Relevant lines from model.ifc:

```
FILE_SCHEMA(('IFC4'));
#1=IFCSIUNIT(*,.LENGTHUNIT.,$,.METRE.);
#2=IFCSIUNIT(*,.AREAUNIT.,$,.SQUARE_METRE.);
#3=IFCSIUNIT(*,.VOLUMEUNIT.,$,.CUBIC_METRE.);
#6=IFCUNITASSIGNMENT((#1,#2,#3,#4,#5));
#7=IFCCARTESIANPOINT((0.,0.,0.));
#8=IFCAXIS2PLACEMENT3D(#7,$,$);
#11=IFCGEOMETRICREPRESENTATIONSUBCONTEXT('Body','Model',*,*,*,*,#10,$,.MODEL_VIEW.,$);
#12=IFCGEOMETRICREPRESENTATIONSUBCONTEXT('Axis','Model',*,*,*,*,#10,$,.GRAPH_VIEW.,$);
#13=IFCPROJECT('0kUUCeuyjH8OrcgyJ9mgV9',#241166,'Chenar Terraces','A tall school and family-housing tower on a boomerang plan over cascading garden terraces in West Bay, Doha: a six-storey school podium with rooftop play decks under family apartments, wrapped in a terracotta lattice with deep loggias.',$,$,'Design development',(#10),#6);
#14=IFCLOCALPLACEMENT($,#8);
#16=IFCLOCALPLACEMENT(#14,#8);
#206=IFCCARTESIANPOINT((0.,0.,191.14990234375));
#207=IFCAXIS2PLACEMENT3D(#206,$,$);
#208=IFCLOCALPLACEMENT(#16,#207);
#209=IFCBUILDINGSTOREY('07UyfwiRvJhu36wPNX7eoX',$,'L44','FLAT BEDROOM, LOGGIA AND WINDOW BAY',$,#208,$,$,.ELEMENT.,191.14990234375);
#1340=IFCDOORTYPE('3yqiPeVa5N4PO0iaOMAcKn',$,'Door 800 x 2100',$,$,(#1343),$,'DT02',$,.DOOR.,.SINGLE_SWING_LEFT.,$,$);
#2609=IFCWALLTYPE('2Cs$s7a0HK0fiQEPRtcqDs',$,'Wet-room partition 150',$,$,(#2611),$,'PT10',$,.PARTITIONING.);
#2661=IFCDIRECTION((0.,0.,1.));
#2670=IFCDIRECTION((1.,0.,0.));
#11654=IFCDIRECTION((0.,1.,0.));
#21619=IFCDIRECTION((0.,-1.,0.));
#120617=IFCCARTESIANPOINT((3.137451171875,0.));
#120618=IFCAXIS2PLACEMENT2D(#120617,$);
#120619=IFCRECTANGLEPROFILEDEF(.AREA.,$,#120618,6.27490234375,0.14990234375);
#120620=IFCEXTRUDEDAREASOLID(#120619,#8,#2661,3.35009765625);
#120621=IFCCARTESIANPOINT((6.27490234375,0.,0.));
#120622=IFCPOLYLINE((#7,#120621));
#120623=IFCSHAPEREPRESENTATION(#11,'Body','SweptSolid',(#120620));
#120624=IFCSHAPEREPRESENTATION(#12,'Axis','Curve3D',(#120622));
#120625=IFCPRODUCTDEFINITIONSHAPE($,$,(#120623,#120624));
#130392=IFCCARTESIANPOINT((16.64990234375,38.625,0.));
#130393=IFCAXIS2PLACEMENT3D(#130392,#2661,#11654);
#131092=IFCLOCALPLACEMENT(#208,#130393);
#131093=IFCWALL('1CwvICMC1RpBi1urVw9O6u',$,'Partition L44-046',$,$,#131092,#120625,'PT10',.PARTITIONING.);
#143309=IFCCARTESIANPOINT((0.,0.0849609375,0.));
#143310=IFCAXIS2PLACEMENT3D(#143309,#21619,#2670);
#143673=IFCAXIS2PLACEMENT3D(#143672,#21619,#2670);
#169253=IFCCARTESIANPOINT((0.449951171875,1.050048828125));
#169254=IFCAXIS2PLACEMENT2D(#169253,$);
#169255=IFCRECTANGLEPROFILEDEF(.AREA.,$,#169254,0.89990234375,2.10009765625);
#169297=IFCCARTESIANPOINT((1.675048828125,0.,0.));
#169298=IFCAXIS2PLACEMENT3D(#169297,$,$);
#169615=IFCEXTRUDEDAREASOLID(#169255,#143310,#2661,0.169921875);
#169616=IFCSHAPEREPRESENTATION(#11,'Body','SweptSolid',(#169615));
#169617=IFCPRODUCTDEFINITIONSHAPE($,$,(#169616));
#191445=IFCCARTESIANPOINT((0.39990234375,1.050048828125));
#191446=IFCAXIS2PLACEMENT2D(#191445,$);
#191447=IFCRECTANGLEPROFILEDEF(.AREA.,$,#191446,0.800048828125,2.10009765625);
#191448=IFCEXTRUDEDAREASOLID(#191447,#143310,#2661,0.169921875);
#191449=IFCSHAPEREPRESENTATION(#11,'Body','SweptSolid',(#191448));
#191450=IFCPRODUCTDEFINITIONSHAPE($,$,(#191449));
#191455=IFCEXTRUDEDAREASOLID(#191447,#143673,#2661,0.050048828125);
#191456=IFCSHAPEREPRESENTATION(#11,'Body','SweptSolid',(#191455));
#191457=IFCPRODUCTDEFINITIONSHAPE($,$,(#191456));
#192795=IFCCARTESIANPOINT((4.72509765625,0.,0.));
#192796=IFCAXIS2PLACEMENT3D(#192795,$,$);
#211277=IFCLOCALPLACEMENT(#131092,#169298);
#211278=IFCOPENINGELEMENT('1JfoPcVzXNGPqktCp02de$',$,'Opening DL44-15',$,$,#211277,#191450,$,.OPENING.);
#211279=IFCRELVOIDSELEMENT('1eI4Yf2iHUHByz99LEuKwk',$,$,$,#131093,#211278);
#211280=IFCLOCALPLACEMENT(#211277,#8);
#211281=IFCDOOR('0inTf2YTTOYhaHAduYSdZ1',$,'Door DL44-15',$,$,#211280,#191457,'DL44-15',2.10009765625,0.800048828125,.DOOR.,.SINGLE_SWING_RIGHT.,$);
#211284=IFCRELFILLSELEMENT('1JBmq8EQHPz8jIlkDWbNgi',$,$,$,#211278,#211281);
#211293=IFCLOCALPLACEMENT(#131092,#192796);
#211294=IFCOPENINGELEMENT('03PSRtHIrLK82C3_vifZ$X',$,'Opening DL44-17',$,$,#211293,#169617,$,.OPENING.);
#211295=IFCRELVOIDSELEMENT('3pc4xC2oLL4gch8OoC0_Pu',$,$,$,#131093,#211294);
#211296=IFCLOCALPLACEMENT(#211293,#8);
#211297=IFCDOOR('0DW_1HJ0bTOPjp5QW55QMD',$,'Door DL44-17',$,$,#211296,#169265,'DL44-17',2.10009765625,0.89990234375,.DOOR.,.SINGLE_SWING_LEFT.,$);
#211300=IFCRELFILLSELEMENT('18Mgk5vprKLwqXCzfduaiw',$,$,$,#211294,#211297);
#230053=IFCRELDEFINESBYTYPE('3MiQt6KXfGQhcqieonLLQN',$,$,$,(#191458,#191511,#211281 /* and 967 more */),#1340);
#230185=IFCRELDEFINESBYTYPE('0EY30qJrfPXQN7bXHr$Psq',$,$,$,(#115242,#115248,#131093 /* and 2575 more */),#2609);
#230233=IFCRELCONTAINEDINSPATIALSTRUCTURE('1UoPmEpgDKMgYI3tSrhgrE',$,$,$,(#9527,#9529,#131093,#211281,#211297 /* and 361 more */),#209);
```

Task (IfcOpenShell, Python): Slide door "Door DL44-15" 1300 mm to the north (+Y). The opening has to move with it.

```python
import ifcopenshell
import ifcopenshell.api.geometry
import ifcopenshell.util.placement

model = ifcopenshell.open("model.ifc")

door = model.by_guid("0inTf2YTTOYhaHAduYSdZ1")
opening = door.FillsVoids[0].RelatingOpeningElement
wall = opening.VoidsElements[0].RelatingBuildingElement

wall_matrix = ifcopenshell.util.placement.get_local_placement(wall.ObjectPlacement)
shift = wall_matrix[:3, 0] * 1.3
before = ifcopenshell.util.placement.get_local_placement(door.ObjectPlacement)[:3, 3].copy()

# The door is placed relative to its opening, so it follows when the opening moves.
matrix = ifcopenshell.util.placement.get_local_placement(opening.ObjectPlacement)
matrix[:3, 3] += shift
ifcopenshell.api.geometry.edit_object_placement(
    model, product=opening, matrix=matrix, is_si=False, should_transform_children=True
)

after = ifcopenshell.util.placement.get_local_placement(door.ObjectPlacement)[:3, 3]
print("door moved by", (after - before).round(3) + 0.0)

model.write("model_updated.ifc")
```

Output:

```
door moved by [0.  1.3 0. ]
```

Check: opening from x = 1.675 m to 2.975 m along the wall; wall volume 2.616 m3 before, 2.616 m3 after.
